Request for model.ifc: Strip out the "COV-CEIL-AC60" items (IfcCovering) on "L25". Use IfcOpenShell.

First a look at what the model holds.

```python
import ifcopenshell
import ifcopenshell.util.element

model = ifcopenshell.open("model.ifc")
print(model.schema)
storey = next(s for s in model.by_type("IfcBuildingStorey") if s.Name == "L25")
coverings = [e for e in ifcopenshell.util.element.get_decomposition(storey) if e.is_a("IfcCovering")]
seen = {}
for e in coverings:
    element_type = ifcopenshell.util.element.get_type(e)
    name = element_type.Name if element_type not in (None, e) else None
    seen[name] = seen.get(name, 0) + 1
for name, count in sorted(seen.items(), key=str):
    print(count, "x", name)
```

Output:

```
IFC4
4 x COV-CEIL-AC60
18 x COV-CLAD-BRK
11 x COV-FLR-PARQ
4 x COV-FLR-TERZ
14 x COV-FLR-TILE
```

```python
import ifcopenshell
import ifcopenshell.api.root
import ifcopenshell.util.element

model = ifcopenshell.open("model.ifc")

storey = next(s for s in model.by_type("IfcBuildingStorey") if s.Name == "L25")
coverings = [e for e in ifcopenshell.util.element.get_decomposition(storey) if e.is_a("IfcCovering")]
targets = [e for e in coverings if (t := ifcopenshell.util.element.get_type(e)) not in (None, e) and t.Name == "COV-CEIL-AC60"]

for e in targets:
    ifcopenshell.api.root.remove_product(model, product=e)
print(len(targets), "removed")

model.write("model_edited.ifc")
```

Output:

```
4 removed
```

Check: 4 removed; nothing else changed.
